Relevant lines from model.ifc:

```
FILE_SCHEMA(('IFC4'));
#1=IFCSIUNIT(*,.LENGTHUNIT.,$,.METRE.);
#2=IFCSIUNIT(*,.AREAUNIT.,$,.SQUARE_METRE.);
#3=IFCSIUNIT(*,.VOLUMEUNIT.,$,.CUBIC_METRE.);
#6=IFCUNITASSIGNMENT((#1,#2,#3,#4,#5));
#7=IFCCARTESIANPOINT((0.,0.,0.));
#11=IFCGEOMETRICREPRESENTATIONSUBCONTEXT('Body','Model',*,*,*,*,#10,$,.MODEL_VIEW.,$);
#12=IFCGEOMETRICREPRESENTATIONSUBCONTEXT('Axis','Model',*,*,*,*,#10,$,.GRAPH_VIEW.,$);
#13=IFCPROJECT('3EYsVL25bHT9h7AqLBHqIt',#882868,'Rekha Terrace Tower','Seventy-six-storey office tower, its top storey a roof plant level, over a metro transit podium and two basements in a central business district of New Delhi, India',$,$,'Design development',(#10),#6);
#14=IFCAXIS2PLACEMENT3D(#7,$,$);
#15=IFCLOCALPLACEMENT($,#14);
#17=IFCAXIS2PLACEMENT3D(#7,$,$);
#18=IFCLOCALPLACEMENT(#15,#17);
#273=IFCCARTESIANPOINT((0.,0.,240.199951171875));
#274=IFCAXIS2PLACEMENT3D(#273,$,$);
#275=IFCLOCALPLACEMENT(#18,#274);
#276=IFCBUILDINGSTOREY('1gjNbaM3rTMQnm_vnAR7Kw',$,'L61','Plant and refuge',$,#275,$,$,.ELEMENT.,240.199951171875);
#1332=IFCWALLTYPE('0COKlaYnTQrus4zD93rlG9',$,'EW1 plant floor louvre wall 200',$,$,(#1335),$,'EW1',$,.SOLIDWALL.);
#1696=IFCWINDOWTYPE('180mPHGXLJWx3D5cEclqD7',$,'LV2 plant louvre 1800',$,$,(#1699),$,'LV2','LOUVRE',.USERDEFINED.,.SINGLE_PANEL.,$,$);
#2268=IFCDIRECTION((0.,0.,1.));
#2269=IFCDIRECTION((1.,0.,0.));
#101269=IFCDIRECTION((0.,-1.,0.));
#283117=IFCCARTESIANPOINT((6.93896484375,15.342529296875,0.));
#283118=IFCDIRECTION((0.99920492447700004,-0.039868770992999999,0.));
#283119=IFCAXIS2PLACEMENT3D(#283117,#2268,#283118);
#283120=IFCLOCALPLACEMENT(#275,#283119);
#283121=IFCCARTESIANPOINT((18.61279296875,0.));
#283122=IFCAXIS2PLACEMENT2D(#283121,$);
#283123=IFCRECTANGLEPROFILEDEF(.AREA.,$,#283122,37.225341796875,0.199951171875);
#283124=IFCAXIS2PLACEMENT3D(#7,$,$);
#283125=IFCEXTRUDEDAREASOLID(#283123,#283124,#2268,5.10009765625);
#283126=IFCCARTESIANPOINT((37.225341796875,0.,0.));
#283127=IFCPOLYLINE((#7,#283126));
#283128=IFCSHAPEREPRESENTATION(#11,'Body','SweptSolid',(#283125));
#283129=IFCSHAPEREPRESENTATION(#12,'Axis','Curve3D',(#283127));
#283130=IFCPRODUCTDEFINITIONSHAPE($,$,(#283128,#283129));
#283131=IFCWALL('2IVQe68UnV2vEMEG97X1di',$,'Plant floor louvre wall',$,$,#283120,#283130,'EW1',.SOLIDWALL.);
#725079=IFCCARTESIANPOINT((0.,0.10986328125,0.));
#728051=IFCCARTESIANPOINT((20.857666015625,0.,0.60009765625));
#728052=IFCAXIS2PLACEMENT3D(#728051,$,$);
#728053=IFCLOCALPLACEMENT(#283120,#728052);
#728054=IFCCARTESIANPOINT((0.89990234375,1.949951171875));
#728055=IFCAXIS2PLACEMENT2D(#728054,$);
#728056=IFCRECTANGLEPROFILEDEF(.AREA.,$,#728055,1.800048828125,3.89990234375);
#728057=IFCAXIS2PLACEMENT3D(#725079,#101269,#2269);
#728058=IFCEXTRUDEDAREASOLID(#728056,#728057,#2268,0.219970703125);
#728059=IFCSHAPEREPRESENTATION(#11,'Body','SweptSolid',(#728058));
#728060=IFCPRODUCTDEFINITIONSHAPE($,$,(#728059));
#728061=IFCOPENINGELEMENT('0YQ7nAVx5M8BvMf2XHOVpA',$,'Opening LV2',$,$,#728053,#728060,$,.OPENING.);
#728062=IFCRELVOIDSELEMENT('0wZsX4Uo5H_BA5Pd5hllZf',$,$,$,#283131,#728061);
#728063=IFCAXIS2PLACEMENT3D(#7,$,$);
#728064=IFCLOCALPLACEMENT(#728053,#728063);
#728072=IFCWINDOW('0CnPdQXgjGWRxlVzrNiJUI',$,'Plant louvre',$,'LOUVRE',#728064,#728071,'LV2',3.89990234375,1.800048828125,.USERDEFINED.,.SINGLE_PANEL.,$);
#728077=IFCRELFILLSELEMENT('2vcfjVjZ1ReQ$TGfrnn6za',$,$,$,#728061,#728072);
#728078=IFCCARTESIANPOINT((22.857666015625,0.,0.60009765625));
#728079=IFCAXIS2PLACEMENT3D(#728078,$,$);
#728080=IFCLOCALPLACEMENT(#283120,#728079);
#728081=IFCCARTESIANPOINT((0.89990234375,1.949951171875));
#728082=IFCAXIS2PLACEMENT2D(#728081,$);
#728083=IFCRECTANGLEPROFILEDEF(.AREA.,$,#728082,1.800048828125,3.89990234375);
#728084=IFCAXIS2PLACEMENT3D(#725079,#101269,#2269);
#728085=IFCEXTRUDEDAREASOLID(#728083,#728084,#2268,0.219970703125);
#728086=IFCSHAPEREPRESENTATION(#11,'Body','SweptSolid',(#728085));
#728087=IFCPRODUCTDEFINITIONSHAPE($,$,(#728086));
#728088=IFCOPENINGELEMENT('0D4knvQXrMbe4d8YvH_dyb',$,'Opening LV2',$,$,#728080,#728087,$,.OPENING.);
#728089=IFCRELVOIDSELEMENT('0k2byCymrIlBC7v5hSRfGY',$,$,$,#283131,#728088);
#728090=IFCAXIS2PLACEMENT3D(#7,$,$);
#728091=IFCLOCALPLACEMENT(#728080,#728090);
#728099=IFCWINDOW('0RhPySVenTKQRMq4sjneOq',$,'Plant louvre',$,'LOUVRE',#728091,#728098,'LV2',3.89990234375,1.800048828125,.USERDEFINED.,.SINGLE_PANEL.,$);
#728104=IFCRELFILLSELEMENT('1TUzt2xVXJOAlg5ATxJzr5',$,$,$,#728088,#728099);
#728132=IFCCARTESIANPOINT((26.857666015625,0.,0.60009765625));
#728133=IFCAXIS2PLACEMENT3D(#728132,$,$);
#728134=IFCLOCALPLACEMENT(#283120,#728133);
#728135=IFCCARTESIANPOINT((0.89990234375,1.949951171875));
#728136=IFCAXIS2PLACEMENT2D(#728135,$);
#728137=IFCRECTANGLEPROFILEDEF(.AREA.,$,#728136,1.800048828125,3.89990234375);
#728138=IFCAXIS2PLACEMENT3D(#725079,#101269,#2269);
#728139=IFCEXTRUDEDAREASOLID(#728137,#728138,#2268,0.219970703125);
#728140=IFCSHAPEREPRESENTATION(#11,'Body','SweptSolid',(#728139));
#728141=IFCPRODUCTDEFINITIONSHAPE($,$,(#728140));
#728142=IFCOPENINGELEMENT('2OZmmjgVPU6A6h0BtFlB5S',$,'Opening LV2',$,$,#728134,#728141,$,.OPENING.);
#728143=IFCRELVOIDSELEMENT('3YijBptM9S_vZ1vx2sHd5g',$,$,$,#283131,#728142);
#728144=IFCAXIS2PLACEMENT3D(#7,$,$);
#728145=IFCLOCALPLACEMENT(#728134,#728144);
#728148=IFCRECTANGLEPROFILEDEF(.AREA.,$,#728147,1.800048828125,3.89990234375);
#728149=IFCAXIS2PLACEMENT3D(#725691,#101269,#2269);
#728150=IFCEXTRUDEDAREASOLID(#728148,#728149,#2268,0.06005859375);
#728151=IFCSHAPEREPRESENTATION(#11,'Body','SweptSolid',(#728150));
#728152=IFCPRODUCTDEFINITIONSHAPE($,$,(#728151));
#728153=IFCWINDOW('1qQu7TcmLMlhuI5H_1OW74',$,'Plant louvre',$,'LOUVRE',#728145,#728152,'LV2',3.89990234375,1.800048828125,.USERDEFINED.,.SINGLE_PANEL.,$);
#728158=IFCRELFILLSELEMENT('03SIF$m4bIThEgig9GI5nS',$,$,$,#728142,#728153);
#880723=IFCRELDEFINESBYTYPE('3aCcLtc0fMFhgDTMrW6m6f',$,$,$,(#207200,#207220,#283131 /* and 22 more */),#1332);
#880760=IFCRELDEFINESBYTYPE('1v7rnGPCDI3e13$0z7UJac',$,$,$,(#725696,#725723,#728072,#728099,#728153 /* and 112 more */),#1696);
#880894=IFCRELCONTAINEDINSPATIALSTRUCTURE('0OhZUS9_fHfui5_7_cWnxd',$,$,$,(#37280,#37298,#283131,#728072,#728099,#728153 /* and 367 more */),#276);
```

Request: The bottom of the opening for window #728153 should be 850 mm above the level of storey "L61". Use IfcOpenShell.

```python
import numpy as np
import ifcopenshell
import ifcopenshell.api.geometry
import ifcopenshell.geom
import ifcopenshell.util.element
import ifcopenshell.util.placement
import ifcopenshell.util.shape
import ifcopenshell.util.unit

model = ifcopenshell.open("model.ifc")
unit_scale = ifcopenshell.util.unit.calculate_unit_scale(model)

window = model.by_guid("1qQu7TcmLMlhuI5H_1OW74")
opening = window.FillsVoids[0].RelatingOpeningElement
storey = ifcopenshell.util.element.get_container(window, ifc_class="IfcBuildingStorey")
level = ifcopenshell.util.placement.get_local_placement(storey.ObjectPlacement)[2, 3]

# The opening's origin need not be at the sill, so measure its lowest point.
shape = ifcopenshell.geom.create_shape(ifcopenshell.geom.settings(), opening)
bottom = ifcopenshell.util.shape.get_shape_bottom_elevation(shape, shape.geometry) / unit_scale
dz = level + 0.85 / unit_scale - bottom

shift = np.array([0.0, 0.0, dz])
# The window is placed relative to its opening, so it follows when the opening moves.
matrix = ifcopenshell.util.placement.get_local_placement(opening.ObjectPlacement)
matrix[:3, 3] += shift
ifcopenshell.api.geometry.edit_object_placement(
    model, product=opening, matrix=matrix, is_si=False, should_transform_children=True
)

print(f"moved by {dz * unit_scale:+.3f} m")

model.write("model-out.ifc")
```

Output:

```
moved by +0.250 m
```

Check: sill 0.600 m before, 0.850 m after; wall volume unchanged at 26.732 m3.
